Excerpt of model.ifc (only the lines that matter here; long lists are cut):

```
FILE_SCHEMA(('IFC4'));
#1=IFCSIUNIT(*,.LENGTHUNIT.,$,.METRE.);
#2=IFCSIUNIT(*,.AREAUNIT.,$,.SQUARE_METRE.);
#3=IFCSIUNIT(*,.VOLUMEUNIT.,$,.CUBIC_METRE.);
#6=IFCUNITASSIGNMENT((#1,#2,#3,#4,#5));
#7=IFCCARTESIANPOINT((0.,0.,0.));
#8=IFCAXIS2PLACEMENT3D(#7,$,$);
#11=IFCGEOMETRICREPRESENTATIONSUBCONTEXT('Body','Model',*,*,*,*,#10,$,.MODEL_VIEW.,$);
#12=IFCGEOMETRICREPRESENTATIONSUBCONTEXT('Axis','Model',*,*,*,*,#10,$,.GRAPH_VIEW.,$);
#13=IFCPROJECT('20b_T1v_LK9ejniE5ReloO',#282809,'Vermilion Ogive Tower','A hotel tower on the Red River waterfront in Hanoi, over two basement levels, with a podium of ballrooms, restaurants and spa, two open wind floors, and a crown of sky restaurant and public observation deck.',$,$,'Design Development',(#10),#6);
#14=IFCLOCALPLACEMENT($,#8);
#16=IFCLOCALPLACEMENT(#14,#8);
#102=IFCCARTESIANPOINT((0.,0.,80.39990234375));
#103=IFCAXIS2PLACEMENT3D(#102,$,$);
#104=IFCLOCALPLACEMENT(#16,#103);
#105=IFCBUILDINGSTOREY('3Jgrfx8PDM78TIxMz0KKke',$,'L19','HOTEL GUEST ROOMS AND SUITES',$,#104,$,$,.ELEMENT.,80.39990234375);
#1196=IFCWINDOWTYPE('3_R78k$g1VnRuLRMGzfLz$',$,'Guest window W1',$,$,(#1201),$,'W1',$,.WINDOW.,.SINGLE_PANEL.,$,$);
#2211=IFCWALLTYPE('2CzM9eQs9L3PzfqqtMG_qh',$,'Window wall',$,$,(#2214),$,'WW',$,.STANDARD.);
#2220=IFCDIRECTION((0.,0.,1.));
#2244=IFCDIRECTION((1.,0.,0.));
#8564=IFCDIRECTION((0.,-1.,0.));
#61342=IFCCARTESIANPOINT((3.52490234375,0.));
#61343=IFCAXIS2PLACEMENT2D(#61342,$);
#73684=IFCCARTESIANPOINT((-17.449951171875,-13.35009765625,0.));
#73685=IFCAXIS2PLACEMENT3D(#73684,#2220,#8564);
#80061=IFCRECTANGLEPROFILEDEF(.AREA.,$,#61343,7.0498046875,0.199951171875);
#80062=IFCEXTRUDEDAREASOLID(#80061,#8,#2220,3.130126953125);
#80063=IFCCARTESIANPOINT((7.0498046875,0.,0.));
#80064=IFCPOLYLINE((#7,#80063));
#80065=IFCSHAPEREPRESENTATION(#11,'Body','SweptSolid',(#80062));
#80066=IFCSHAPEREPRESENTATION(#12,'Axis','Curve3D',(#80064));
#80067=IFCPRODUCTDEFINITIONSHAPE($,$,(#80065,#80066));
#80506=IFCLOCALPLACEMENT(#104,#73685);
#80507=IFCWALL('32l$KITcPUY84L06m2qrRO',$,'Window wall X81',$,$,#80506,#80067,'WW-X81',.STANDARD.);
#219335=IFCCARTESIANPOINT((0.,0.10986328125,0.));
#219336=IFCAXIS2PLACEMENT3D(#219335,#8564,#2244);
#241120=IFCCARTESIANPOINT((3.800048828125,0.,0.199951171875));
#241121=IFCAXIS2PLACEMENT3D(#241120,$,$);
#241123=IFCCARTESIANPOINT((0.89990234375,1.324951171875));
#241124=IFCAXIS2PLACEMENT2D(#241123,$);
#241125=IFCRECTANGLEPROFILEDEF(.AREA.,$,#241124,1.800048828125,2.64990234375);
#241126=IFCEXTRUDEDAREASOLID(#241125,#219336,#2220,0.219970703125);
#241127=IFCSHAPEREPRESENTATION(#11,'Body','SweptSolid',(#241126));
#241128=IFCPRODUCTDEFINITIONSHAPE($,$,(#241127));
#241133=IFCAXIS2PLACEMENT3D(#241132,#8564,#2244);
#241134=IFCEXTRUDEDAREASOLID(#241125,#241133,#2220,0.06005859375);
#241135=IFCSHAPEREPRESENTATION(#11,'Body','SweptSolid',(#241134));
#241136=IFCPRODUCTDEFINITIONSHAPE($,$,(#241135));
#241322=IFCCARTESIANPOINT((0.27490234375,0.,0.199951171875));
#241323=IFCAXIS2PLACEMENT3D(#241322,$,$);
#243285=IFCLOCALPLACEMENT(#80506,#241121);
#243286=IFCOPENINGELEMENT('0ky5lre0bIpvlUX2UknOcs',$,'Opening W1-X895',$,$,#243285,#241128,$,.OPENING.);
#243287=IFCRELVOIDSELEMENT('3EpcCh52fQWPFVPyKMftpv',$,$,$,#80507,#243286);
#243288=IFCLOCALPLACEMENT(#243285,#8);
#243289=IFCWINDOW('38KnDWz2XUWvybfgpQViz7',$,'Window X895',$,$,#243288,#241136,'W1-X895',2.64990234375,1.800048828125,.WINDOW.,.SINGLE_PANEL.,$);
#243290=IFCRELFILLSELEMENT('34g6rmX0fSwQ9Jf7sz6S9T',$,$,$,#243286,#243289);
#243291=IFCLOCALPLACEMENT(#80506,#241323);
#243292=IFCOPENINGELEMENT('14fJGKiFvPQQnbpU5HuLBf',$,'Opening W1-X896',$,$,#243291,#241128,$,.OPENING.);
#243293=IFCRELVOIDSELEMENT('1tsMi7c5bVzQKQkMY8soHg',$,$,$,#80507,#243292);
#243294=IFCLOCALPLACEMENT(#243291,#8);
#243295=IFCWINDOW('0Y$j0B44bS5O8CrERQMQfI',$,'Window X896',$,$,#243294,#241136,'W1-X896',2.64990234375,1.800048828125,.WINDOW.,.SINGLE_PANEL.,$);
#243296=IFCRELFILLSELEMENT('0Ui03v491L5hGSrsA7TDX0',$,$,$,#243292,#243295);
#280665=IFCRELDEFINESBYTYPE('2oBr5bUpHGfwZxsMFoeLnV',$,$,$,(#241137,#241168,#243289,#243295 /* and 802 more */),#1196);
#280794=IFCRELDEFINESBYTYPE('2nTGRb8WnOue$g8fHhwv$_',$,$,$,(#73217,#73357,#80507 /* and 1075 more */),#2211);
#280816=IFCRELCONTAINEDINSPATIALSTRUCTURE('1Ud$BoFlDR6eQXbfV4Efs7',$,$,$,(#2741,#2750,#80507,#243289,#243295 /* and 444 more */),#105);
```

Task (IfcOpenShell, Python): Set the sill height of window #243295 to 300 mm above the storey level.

```python
import numpy as np
import ifcopenshell
import ifcopenshell.api.geometry
import ifcopenshell.geom
import ifcopenshell.util.element
import ifcopenshell.util.placement
import ifcopenshell.util.shape
import ifcopenshell.util.unit

model = ifcopenshell.open("model.ifc")
unit_scale = ifcopenshell.util.unit.calculate_unit_scale(model)

window = model.by_id(243295)
opening = window.FillsVoids[0].RelatingOpeningElement
storey = ifcopenshell.util.element.get_container(window, ifc_class="IfcBuildingStorey")
level = ifcopenshell.util.placement.get_local_placement(storey.ObjectPlacement)[2, 3]

# The opening's origin need not be at the sill, so measure its lowest point.
shape = ifcopenshell.geom.create_shape(ifcopenshell.geom.settings(), opening)
bottom = ifcopenshell.util.shape.get_shape_bottom_elevation(shape, shape.geometry) / unit_scale
dz = level + 0.3 / unit_scale - bottom

shift = np.array([0.0, 0.0, dz])
# The window is placed relative to its opening, so it follows when the opening moves.
matrix = ifcopenshell.util.placement.get_local_placement(opening.ObjectPlacement)
matrix[:3, 3] += shift
ifcopenshell.api.geometry.edit_object_placement(
    model, product=opening, matrix=matrix, is_si=False, should_transform_children=True
)

print(f"moved by {dz * unit_scale:+.3f} m")

model.write("model_v2.ifc")
```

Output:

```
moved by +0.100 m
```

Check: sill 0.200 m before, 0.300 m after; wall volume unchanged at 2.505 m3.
